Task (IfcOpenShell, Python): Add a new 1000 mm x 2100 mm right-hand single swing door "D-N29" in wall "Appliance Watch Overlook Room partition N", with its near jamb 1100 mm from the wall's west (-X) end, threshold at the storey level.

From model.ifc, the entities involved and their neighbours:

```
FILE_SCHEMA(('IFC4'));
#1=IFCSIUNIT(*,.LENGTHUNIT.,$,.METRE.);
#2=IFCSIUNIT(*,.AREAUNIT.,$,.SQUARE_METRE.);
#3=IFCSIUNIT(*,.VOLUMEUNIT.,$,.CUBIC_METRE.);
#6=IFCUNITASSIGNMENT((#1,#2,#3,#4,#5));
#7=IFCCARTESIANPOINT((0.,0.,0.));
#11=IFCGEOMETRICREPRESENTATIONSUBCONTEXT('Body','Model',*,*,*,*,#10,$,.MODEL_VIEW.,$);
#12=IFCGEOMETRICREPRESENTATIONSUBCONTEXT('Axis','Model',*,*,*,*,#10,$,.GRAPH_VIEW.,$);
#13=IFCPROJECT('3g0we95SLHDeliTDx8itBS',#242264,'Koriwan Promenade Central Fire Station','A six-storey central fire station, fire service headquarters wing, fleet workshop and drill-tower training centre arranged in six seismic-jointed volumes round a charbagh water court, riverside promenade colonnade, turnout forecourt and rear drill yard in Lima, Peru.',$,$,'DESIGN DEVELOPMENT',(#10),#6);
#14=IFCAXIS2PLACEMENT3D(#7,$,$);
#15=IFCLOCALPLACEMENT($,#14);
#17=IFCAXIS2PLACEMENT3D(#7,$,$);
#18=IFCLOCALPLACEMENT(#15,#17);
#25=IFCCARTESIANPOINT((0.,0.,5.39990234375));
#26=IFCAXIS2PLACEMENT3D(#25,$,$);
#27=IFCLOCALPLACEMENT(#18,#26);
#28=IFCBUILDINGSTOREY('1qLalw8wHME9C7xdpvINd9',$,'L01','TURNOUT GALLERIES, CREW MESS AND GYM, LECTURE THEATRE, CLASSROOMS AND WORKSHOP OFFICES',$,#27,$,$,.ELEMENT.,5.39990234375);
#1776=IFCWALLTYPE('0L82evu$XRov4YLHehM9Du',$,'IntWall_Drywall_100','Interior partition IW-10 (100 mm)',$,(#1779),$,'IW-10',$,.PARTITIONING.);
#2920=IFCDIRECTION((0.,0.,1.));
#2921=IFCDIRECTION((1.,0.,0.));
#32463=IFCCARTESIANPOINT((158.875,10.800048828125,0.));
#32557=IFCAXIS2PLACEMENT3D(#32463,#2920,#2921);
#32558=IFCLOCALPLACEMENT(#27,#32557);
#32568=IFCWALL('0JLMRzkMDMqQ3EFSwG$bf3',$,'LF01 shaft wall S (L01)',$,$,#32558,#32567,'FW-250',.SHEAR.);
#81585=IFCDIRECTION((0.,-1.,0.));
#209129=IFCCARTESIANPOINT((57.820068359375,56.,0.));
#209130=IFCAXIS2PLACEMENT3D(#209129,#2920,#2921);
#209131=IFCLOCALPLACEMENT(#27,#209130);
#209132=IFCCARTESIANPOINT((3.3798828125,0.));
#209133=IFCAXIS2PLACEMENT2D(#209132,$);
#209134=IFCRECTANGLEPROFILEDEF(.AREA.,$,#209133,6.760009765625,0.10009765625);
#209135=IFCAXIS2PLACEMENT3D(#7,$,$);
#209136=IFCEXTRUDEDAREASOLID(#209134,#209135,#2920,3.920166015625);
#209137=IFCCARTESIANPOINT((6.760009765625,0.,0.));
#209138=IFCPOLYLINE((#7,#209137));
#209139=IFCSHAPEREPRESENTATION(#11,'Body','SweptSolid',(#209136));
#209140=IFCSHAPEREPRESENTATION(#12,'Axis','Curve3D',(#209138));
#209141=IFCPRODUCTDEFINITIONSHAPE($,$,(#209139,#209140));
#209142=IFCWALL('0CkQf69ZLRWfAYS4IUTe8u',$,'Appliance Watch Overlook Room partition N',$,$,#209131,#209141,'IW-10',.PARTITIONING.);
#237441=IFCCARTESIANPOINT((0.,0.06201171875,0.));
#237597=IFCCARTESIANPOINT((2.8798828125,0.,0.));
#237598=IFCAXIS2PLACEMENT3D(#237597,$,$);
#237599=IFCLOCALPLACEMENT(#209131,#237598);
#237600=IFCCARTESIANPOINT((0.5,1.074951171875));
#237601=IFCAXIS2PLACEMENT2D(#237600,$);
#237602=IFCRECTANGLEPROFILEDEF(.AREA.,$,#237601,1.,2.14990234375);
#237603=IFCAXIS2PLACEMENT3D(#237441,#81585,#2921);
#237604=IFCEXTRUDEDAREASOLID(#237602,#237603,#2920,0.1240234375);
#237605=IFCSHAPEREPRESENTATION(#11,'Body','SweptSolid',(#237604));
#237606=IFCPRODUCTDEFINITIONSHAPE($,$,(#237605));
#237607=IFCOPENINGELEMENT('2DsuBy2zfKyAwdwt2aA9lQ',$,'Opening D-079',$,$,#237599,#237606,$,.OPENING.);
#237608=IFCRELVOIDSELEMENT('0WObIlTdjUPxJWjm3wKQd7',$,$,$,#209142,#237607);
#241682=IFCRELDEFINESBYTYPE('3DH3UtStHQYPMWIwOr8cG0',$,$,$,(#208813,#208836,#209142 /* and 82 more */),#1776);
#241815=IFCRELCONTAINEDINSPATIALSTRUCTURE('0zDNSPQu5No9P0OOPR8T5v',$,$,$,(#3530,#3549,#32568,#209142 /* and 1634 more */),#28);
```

```python
import numpy as np
import ifcopenshell
import ifcopenshell.api.feature
import ifcopenshell.api.geometry
import ifcopenshell.api.root
import ifcopenshell.api.spatial
import ifcopenshell.geom
import ifcopenshell.util.element
import ifcopenshell.util.placement
import ifcopenshell.util.representation
import ifcopenshell.util.shape
import ifcopenshell.util.unit

model = ifcopenshell.open("model.ifc")
unit_scale = ifcopenshell.util.unit.calculate_unit_scale(model)
settings = ifcopenshell.geom.settings()


def volume(element):
    """Net volume in cubic metres, openings subtracted."""
    shape = ifcopenshell.geom.create_shape(settings, element)
    return ifcopenshell.util.shape.get_volume(shape.geometry)


wall = model.by_guid("0CkQf69ZLRWfAYS4IUTe8u")
storey = ifcopenshell.util.element.get_container(wall, ifc_class="IfcBuildingStorey")
context = ifcopenshell.util.representation.get_context(model, "Model", "Body", "MODEL_VIEW")
before = volume(wall)

width, height, from_end, sill = 1, 2.1, 1.1, 0.0  # metres

# The wall runs along its own X axis, and the end named is its -X end.
wall_shape = ifcopenshell.geom.create_shape(settings, wall)
x, y, z = ifcopenshell.util.shape.get_vertices(wall_shape.geometry).T
start = x.min() + from_end
face, thickness = float(y.min()), float(y.max() - y.min())
wall_matrix = ifcopenshell.util.placement.get_local_placement(wall.ObjectPlacement)
level = ifcopenshell.util.placement.get_local_placement(storey.ObjectPlacement)[2, 3]


def in_wall(x, y):
    """Placement at x, y metres in the wall's axes, at sill height."""
    matrix = wall_matrix.copy()
    matrix[:, 3] = wall_matrix @ np.array([x / unit_scale, y / unit_scale, 0.0, 1.0])
    matrix[2, 3] = level + sill / unit_scale
    return matrix


# Opening: a box that overshoots both wall faces by 50 mm.
opening = ifcopenshell.api.root.create_entity(model, ifc_class="IfcOpeningElement", predefined_type="OPENING")
box = ifcopenshell.api.geometry.add_wall_representation(
    model, context=context, length=width, height=height, thickness=thickness + 0.1
)
ifcopenshell.api.geometry.assign_representation(model, product=opening, representation=box)
ifcopenshell.api.geometry.edit_object_placement(model, product=opening, matrix=in_wall(start, face - 0.05), is_si=False)
ifcopenshell.api.feature.add_feature(model, feature=opening, element=wall)

door = ifcopenshell.api.root.create_entity(model, ifc_class="IfcDoor", name="D-N29", predefined_type="DOOR")
door.OverallWidth, door.OverallHeight = width / unit_scale, height / unit_scale
door.OperationType = "SINGLE_SWING_RIGHT"
body = ifcopenshell.api.geometry.add_door_representation(
    model,
    context=context,
    overall_width=door.OverallWidth,
    overall_height=door.OverallHeight,
    operation_type="SINGLE_SWING_RIGHT",
    lining_properties={"LiningDepth": thickness / unit_scale, "ThresholdDepth": thickness / unit_scale},
)
ifcopenshell.api.geometry.assign_representation(model, product=door, representation=body)
ifcopenshell.api.spatial.assign_container(model, products=[door], relating_structure=storey)
ifcopenshell.api.feature.add_filling(model, opening=opening, element=door)

# The lining spans the wall, so the door starts at the wall face.
ifcopenshell.api.geometry.edit_object_placement(model, product=door, matrix=in_wall(start, face), is_si=False)

after = volume(wall)

print(f"wall volume {before:.3f} -> {after:.3f} m3")

model.write("model-out.ifc")
```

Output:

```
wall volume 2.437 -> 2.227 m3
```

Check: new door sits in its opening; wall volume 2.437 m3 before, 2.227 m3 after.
